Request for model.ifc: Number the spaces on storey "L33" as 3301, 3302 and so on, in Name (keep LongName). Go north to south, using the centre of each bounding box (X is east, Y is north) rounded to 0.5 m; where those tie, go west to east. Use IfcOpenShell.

First a look at what the model holds.

```python
import ifcopenshell
import ifcopenshell.util.element
import ifcopenshell.util.placement

model = ifcopenshell.open("model.ifc")
print(model.schema)
storey = next(s for s in model.by_type("IfcBuildingStorey") if s.Name == "L33")
spaces = [e for e in ifcopenshell.util.element.get_decomposition(storey) if e.is_a("IfcSpace")]
for e in sorted(spaces, key=lambda e: e.id()):
    origin = ifcopenshell.util.placement.get_local_placement(e.ObjectPlacement)[:3, 3]
    print(e.id(), e.Name, e.LongName, origin.round(2) + 0.0, sep=" | ")
```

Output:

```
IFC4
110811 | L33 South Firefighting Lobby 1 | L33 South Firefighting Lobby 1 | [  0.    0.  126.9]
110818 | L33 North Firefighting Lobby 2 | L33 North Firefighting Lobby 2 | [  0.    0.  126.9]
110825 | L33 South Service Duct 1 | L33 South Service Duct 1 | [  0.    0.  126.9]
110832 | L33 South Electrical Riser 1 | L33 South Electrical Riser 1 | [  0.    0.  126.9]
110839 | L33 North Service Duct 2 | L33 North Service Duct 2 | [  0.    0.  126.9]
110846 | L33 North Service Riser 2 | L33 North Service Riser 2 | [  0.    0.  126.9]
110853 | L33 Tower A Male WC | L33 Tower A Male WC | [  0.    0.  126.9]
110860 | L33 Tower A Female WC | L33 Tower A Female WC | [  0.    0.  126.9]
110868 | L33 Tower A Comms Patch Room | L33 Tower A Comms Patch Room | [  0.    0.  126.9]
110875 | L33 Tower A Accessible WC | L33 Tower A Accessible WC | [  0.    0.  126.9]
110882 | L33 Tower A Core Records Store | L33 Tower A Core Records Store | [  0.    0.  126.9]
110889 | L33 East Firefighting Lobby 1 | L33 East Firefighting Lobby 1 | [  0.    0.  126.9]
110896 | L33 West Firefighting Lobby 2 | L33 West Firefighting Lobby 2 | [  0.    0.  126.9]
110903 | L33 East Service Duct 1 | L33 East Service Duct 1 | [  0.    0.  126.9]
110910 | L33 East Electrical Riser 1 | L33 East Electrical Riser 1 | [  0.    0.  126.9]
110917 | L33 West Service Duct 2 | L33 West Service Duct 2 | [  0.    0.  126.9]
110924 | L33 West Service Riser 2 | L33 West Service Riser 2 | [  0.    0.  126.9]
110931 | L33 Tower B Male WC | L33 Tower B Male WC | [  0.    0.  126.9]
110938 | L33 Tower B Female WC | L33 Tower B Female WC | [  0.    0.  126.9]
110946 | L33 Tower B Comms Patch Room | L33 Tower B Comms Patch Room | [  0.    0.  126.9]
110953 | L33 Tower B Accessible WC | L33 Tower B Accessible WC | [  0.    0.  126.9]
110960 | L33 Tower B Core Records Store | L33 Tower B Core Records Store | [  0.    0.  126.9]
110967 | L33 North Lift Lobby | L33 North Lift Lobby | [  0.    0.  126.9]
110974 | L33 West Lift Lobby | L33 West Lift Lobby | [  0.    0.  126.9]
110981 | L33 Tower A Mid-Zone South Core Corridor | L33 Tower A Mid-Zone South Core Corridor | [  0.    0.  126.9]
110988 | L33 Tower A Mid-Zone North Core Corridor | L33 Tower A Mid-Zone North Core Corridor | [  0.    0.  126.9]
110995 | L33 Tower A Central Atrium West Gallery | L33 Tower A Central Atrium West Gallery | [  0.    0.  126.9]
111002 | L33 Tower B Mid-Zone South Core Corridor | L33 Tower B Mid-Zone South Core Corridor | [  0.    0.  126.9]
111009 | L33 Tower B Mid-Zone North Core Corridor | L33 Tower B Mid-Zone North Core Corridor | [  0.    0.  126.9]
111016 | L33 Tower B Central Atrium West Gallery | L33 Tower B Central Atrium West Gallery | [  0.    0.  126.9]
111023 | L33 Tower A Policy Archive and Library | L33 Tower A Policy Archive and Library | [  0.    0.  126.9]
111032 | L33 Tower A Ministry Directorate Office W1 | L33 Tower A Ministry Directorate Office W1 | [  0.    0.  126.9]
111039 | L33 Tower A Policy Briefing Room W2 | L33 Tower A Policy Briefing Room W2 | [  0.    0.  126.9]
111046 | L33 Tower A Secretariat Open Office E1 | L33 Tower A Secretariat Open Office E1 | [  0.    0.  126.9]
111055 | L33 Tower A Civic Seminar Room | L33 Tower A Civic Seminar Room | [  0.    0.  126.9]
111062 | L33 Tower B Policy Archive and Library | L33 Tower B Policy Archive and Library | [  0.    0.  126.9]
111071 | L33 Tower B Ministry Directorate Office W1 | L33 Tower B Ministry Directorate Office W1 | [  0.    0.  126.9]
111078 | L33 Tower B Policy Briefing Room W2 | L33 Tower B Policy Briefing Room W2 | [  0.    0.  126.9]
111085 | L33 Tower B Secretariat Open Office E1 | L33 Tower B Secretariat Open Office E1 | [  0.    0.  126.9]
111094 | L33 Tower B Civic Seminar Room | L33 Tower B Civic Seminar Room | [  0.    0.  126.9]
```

```python
import ifcopenshell
import ifcopenshell.geom
import ifcopenshell.util.element
import ifcopenshell.util.shape

model = ifcopenshell.open("model.ifc")
settings = ifcopenshell.geom.settings()
settings.set("use-world-coords", True)


def centre(element):
    shape = ifcopenshell.geom.create_shape(settings, element)
    return ifcopenshell.util.shape.get_bbox_centroid(shape.geometry)


storey = next(s for s in model.by_type("IfcBuildingStorey") if s.Name == "L33")
spaces = [e for e in ifcopenshell.util.element.get_decomposition(storey) if e.is_a("IfcSpace")]

# Insertion points can sit at a corner or the storey origin, so sort by the geometry (in metres).
centres = {e: centre(e) for e in spaces}
spaces.sort(key=lambda e: (-round(centres[e][1] / 0.5), centres[e][0]))

for i, e in enumerate(spaces, start=1):
    number = f"33{i:02d}"
    e.Name = number
    print(e.id(), number)

model.write("model_v2.ifc")
```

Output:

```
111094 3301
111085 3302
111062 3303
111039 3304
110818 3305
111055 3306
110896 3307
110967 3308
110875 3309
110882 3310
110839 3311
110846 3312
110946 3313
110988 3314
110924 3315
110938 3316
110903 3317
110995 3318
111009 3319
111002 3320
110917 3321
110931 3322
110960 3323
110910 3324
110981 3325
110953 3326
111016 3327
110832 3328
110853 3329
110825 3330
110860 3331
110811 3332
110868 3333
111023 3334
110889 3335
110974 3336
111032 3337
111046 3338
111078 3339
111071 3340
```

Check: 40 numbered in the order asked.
